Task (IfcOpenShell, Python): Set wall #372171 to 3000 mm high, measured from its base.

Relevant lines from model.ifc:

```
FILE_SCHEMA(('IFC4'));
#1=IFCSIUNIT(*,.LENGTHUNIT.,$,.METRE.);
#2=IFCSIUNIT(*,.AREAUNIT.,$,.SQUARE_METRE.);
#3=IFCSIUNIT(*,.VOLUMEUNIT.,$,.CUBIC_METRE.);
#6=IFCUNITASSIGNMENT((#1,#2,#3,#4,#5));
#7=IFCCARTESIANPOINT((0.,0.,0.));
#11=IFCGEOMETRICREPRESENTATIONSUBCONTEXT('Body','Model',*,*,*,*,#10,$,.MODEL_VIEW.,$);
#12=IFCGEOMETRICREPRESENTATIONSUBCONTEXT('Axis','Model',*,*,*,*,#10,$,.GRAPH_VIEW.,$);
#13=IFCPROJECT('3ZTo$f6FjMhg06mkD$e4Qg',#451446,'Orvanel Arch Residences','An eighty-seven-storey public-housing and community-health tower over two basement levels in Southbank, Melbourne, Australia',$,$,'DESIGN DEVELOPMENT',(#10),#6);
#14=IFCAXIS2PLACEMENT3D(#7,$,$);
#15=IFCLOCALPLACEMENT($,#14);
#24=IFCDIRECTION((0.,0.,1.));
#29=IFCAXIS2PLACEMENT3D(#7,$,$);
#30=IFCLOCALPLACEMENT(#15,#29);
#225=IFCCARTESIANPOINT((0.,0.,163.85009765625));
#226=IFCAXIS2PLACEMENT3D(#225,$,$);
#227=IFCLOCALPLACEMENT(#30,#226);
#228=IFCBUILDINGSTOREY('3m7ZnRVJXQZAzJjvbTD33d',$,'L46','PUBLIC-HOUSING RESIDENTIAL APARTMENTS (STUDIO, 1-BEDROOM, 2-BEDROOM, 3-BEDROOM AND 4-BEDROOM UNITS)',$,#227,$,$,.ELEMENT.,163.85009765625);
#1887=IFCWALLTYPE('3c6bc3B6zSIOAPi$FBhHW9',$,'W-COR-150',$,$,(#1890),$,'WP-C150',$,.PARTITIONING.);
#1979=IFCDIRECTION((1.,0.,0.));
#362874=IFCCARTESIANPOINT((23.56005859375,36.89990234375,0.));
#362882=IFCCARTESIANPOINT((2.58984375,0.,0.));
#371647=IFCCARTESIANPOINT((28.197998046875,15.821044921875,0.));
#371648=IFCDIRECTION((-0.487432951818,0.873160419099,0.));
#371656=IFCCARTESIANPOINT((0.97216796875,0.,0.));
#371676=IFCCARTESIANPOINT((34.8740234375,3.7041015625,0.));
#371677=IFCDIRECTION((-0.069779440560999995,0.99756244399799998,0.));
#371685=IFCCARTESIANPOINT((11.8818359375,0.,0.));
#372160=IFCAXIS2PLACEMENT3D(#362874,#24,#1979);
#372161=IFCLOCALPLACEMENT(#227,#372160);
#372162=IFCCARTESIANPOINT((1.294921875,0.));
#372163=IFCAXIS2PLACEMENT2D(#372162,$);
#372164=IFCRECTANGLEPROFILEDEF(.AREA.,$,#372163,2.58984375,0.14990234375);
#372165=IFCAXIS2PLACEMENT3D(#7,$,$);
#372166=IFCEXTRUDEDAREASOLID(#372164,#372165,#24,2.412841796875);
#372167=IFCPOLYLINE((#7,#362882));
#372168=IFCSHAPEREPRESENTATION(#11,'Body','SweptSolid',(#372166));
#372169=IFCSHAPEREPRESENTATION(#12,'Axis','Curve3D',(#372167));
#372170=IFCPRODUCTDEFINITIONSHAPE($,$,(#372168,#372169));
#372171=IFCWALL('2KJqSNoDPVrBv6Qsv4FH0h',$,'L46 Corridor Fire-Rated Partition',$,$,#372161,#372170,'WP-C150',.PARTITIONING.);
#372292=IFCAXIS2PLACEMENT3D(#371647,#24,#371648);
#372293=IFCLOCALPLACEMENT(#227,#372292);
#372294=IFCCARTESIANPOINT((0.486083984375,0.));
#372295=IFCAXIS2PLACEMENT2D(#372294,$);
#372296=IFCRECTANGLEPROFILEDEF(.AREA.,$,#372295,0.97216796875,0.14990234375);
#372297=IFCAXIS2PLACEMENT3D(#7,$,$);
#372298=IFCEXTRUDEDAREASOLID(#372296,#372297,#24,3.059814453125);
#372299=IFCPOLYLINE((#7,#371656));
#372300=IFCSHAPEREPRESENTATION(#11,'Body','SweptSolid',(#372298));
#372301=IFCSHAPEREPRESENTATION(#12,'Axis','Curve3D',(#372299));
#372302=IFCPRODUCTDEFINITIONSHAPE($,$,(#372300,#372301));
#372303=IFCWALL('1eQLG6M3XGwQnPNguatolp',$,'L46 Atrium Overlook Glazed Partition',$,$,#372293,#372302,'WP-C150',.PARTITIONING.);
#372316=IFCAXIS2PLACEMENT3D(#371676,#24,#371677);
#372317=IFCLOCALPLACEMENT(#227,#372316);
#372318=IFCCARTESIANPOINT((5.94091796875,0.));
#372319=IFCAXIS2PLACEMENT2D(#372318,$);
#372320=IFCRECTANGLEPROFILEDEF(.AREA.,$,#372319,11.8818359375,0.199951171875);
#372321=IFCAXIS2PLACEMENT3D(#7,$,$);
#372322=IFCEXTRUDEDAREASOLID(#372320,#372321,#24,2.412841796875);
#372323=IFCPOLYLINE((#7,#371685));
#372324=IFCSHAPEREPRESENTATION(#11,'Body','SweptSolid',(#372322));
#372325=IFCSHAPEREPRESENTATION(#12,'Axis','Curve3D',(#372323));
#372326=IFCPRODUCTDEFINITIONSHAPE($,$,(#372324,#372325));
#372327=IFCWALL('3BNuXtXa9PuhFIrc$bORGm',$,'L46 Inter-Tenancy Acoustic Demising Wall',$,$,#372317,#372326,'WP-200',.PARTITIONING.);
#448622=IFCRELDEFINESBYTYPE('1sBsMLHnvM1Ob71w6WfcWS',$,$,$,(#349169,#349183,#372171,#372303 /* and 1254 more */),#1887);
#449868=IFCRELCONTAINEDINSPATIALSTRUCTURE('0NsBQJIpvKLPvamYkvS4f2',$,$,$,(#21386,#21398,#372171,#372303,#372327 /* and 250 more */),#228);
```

```python
import ifcopenshell
import ifcopenshell.geom
import ifcopenshell.util.representation
import ifcopenshell.util.shape
import ifcopenshell.util.unit

model = ifcopenshell.open("model.ifc")
unit_scale = ifcopenshell.util.unit.calculate_unit_scale(model)
settings = ifcopenshell.geom.settings()


def volume(element):
    """Net volume in cubic metres, openings subtracted."""
    shape = ifcopenshell.geom.create_shape(settings, element)
    return ifcopenshell.util.shape.get_volume(shape.geometry)


wall = model.by_guid("2KJqSNoDPVrBv6Qsv4FH0h")
before = volume(wall)

body = ifcopenshell.util.representation.get_representation(wall, "Model", "Body")
solid = body.Items[0]
old_height = solid.Depth
solid.Depth = 3 / unit_scale
after = volume(wall)

print(f"height {old_height:g} -> {solid.Depth:g}, volume {before:.3f} -> {after:.3f} m3")

model.write("model-out.ifc")
```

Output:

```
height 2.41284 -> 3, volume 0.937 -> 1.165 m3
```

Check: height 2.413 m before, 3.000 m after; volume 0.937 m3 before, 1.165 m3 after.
